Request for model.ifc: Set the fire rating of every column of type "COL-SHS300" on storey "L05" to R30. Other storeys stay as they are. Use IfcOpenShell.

First a look at what the model holds.

```python
import ifcopenshell
import ifcopenshell.util.element

model = ifcopenshell.open("model.ifc")
print(model.schema)
storey = next(s for s in model.by_type("IfcBuildingStorey") if s.Name == "L05")
columns = [e for e in ifcopenshell.util.element.get_decomposition(storey) if e.is_a("IfcColumn")]
seen = {}
for e in columns:
    element_type = ifcopenshell.util.element.get_type(e)
    key = (element_type.Name if element_type != e and element_type else None, ifcopenshell.util.element.get_pset(e, "Pset_ColumnCommon", "FireRating"))
    seen[key] = seen.get(key, 0) + 1
for (name, value), count in sorted(seen.items(), key=str):
    print(count, "x", name, "|", value)
```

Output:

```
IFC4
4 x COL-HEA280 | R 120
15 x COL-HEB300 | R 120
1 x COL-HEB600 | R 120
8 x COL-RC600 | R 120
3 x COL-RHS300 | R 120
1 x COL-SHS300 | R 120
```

```python
import ifcopenshell
import ifcopenshell.api.pset
import ifcopenshell.util.element

model = ifcopenshell.open("model.ifc")

storey = next(s for s in model.by_type("IfcBuildingStorey") if s.Name == "L05")
columns = [e for e in ifcopenshell.util.element.get_decomposition(storey) if e.is_a("IfcColumn")]

count = 0
for e in columns:
    element_type = ifcopenshell.util.element.get_type(e)
    if element_type in (None, e) or element_type.Name != "COL-SHS300":
        continue
    # add_pset returns the element's existing set when there is one.
    pset = ifcopenshell.api.pset.add_pset(model, product=e, name="Pset_ColumnCommon")
    ifcopenshell.api.pset.edit_pset(model, pset=pset, properties={"FireRating": "R30"})
    count += 1

print(count, "columns updated")

model.write("model_v2.ifc")
```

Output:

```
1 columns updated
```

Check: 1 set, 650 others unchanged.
